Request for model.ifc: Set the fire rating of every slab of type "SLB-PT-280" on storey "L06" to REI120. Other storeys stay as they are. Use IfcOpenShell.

First a look at what the model holds.

```python
import ifcopenshell
import ifcopenshell.util.element

model = ifcopenshell.open("model.ifc")
print(model.schema)
storey = next(s for s in model.by_type("IfcBuildingStorey") if s.Name == "L06")
slabs = [e for e in ifcopenshell.util.element.get_decomposition(storey) if e.is_a("IfcSlab")]
seen = {}
for e in slabs:
    element_type = ifcopenshell.util.element.get_type(e)
    key = (element_type.Name if element_type != e and element_type else None, ifcopenshell.util.element.get_pset(e, "Pset_SlabCommon", "FireRating"))
    seen[key] = seen.get(key, 0) + 1
for (name, value), count in sorted(seen.items(), key=str):
    print(count, "x", name, "|", value)
```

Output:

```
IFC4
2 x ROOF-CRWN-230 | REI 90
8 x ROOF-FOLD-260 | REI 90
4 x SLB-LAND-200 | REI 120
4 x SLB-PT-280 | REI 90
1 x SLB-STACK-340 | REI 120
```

```python
import ifcopenshell
import ifcopenshell.api.pset
import ifcopenshell.util.element

model = ifcopenshell.open("model.ifc")

storey = next(s for s in model.by_type("IfcBuildingStorey") if s.Name == "L06")
slabs = [e for e in ifcopenshell.util.element.get_decomposition(storey) if e.is_a("IfcSlab")]

count = 0
for e in slabs:
    element_type = ifcopenshell.util.element.get_type(e)
    if element_type in (None, e) or element_type.Name != "SLB-PT-280":
        continue
    # add_pset returns the element's existing set when there is one.
    pset = ifcopenshell.api.pset.add_pset(model, product=e, name="Pset_SlabCommon")
    ifcopenshell.api.pset.edit_pset(model, pset=pset, properties={"FireRating": "REI120"})
    count += 1

print(count, "slabs updated")

model.write("model_updated.ifc")
```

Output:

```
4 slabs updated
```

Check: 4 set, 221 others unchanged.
